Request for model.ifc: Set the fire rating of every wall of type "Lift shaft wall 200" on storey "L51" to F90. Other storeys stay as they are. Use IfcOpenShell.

First a look at what the model holds.

```python
import ifcopenshell
import ifcopenshell.util.element

model = ifcopenshell.open("model.ifc")
print(model.schema)
storey = next(s for s in model.by_type("IfcBuildingStorey") if s.Name == "L51")
walls = [e for e in ifcopenshell.util.element.get_decomposition(storey) if e.is_a("IfcWall")]
seen = {}
for e in walls:
    element_type = ifcopenshell.util.element.get_type(e)
    key = (element_type.Name if element_type != e and element_type else None, ifcopenshell.util.element.get_pset(e, "Pset_WallCommon", "FireRating"))
    seen[key] = seen.get(key, 0) + 1
for (name, value), count in sorted(seen.items(), key=str):
    print(count, "x", name, "|", value)
```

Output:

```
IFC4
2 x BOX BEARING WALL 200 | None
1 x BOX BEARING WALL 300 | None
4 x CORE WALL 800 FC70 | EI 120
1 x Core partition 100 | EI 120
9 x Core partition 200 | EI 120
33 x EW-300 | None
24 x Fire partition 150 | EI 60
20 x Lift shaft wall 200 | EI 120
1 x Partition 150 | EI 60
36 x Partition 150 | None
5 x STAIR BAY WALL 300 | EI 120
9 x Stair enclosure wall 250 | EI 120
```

```python
import ifcopenshell
import ifcopenshell.api.pset
import ifcopenshell.util.element

model = ifcopenshell.open("model.ifc")

storey = next(s for s in model.by_type("IfcBuildingStorey") if s.Name == "L51")
walls = [e for e in ifcopenshell.util.element.get_decomposition(storey) if e.is_a("IfcWall")]

count = 0
for e in walls:
    element_type = ifcopenshell.util.element.get_type(e)
    if element_type in (None, e) or element_type.Name != "Lift shaft wall 200":
        continue
    found = ifcopenshell.util.element.get_pset(e, "Pset_WallCommon", should_inherit=False)
    if found:
        pset = model.by_id(found["id"])
        if len(ifcopenshell.util.element.get_elements_by_pset(pset)) > 1:
            pset = ifcopenshell.api.pset.unshare_pset(model, products=[e], pset=pset)[0]
    else:
        pset = ifcopenshell.api.pset.add_pset(model, product=e, name="Pset_WallCommon")
    ifcopenshell.api.pset.edit_pset(model, pset=pset, properties={"FireRating": "F90"})
    count += 1

print(count, "walls updated")

model.write("model_updated.ifc")
```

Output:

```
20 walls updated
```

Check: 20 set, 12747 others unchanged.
